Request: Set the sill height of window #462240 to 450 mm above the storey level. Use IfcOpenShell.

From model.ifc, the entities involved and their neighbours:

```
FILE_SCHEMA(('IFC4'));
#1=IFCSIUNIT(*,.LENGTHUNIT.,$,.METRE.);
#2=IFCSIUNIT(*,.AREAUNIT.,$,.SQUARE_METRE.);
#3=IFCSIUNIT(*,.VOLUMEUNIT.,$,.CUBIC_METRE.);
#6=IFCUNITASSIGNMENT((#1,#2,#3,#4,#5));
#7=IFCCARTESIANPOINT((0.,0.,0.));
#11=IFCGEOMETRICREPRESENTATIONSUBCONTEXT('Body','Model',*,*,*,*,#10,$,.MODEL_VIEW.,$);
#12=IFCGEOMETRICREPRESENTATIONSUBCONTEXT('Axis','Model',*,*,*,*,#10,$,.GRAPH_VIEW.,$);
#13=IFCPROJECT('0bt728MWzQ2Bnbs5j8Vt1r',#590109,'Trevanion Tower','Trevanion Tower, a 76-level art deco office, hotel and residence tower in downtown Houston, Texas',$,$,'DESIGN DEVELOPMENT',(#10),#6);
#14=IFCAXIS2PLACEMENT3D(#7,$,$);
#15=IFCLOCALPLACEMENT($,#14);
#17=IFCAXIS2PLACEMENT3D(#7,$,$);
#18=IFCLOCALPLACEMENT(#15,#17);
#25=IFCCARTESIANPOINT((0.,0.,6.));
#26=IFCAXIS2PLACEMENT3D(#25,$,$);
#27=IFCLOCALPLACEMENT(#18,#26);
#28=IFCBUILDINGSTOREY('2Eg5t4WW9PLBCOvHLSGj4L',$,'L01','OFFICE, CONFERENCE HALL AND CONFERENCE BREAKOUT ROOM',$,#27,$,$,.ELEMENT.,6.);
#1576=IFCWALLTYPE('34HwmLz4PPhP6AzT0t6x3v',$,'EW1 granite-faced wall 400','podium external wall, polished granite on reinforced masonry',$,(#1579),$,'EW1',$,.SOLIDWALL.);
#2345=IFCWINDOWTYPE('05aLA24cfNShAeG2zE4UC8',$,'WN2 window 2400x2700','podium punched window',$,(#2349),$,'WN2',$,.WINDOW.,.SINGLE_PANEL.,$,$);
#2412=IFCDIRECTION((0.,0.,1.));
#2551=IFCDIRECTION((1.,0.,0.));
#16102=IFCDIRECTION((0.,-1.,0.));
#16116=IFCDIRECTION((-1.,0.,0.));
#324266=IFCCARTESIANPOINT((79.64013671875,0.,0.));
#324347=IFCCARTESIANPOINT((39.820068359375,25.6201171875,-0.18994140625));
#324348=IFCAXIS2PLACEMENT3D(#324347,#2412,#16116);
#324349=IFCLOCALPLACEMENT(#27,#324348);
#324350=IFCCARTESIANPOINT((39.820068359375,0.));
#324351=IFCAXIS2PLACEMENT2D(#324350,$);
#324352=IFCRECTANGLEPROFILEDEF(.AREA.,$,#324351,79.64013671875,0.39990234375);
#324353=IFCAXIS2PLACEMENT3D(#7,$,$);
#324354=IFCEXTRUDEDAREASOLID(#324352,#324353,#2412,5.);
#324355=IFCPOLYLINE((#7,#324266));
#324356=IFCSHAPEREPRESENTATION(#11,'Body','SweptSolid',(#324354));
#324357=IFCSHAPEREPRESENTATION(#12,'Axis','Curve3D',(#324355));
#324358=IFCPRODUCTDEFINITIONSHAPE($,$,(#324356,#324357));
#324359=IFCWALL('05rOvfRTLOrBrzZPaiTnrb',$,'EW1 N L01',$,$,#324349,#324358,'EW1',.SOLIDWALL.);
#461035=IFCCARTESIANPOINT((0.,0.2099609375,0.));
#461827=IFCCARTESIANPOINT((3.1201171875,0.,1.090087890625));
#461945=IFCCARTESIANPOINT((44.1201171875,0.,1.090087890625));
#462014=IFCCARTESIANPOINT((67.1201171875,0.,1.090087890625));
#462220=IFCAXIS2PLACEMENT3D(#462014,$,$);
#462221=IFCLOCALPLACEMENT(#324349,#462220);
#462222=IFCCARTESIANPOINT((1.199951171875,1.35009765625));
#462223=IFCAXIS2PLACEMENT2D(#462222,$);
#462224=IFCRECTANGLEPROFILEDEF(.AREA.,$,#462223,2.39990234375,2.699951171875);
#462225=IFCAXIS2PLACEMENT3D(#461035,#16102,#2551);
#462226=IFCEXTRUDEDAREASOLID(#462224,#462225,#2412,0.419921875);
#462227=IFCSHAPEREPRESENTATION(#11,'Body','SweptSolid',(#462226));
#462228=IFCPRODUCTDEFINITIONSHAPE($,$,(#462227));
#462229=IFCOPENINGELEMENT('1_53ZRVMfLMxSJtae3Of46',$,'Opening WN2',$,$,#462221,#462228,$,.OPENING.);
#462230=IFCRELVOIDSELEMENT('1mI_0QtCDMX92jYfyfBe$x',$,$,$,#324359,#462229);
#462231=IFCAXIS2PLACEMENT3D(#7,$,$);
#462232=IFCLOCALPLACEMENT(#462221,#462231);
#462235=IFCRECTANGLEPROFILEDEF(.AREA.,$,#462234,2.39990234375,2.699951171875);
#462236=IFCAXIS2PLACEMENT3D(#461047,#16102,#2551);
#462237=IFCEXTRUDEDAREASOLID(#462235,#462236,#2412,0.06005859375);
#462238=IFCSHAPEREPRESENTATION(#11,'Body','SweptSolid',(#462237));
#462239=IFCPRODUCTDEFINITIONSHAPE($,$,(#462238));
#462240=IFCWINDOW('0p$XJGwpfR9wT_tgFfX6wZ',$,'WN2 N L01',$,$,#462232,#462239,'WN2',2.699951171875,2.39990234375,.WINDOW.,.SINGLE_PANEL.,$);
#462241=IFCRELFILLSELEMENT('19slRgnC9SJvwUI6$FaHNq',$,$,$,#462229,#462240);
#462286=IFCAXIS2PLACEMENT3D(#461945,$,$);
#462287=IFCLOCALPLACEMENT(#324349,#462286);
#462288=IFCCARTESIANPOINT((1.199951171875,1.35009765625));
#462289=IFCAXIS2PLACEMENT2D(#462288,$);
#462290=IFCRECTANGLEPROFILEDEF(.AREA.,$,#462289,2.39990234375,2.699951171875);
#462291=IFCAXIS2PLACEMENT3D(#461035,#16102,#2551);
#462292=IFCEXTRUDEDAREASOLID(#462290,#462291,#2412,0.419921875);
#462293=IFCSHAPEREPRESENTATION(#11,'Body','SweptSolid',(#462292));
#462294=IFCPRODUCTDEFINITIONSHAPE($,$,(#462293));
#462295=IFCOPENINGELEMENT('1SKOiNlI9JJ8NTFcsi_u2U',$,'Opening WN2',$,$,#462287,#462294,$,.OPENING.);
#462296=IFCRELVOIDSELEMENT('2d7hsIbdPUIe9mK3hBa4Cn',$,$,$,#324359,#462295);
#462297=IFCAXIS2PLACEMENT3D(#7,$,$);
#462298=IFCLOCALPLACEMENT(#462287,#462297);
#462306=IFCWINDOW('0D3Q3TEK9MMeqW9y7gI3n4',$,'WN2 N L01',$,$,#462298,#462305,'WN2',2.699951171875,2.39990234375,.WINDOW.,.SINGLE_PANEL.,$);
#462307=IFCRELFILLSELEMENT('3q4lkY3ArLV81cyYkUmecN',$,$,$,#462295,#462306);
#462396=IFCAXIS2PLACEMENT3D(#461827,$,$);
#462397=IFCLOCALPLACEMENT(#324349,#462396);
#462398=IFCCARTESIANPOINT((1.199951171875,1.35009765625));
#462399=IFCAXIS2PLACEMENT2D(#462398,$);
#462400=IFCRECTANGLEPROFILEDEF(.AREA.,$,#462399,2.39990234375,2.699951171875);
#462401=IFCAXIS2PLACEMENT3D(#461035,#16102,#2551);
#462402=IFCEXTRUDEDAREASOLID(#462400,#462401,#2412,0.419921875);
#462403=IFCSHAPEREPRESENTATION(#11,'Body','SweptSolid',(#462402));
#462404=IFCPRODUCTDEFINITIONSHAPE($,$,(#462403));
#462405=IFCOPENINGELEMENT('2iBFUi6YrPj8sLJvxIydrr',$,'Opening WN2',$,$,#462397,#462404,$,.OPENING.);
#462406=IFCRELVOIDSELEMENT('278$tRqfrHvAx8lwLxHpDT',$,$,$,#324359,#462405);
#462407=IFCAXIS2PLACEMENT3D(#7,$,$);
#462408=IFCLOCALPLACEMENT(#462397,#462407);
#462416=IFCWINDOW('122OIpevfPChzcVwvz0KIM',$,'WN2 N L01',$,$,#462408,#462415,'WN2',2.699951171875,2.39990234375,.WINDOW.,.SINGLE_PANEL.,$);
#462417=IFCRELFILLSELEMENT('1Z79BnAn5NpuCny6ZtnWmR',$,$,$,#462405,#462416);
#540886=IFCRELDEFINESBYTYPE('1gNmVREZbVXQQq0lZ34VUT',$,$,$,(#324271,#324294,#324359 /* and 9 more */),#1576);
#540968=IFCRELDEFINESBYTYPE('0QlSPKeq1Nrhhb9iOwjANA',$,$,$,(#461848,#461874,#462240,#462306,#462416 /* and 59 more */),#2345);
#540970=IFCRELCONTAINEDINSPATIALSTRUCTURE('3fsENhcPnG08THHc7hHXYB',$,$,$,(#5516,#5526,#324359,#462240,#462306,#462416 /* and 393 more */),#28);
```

```python
import numpy as np
import ifcopenshell
import ifcopenshell.api.geometry
import ifcopenshell.geom
import ifcopenshell.util.element
import ifcopenshell.util.placement
import ifcopenshell.util.shape
import ifcopenshell.util.unit

model = ifcopenshell.open("model.ifc")
unit_scale = ifcopenshell.util.unit.calculate_unit_scale(model)

window = model.by_guid("0p$XJGwpfR9wT_tgFfX6wZ")
opening = window.FillsVoids[0].RelatingOpeningElement
storey = ifcopenshell.util.element.get_container(window, ifc_class="IfcBuildingStorey")
level = ifcopenshell.util.placement.get_local_placement(storey.ObjectPlacement)[2, 3]

# The opening's origin need not be at the sill, so measure its lowest point.
shape = ifcopenshell.geom.create_shape(ifcopenshell.geom.settings(), opening)
bottom = ifcopenshell.util.shape.get_shape_bottom_elevation(shape, shape.geometry) / unit_scale
dz = level + 0.45 - bottom

shift = np.array([0.0, 0.0, dz])
# The window is placed relative to its opening, so it follows when the opening moves.
matrix = ifcopenshell.util.placement.get_local_placement(opening.ObjectPlacement)
matrix[:3, 3] += shift
ifcopenshell.api.geometry.edit_object_placement(
    model, product=opening, matrix=matrix, is_si=False, should_transform_children=True
)

print(f"moved by {dz * unit_scale:+.3f} m")

model.write("model-out.ifc")
```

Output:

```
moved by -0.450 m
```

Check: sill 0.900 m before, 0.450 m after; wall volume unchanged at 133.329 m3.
